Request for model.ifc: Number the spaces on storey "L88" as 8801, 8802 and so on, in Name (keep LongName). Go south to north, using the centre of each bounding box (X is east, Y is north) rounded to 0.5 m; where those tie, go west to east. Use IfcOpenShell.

First a look at what the model holds.

```python
import ifcopenshell
import ifcopenshell.util.element
import ifcopenshell.util.placement

model = ifcopenshell.open("model.ifc")
print(model.schema)
storey = next(s for s in model.by_type("IfcBuildingStorey") if s.Name == "L88")
spaces = [e for e in ifcopenshell.util.element.get_decomposition(storey) if e.is_a("IfcSpace")]
for e in sorted(spaces, key=lambda e: e.id()):
    origin = ifcopenshell.util.placement.get_local_placement(e.ObjectPlacement)[:3, 3]
    print(e.id(), e.Name, e.LongName, origin.round(2) + 0.0, sep=" | ")
```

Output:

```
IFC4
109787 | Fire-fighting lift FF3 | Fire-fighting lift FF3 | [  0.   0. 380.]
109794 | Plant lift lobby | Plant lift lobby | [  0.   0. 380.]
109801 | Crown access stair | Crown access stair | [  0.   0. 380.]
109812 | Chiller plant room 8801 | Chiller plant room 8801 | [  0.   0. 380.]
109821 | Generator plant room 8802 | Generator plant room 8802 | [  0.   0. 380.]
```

```python
import ifcopenshell
import ifcopenshell.geom
import ifcopenshell.util.element
import ifcopenshell.util.shape

model = ifcopenshell.open("model.ifc")
settings = ifcopenshell.geom.settings()
settings.set("use-world-coords", True)


def centre(element):
    shape = ifcopenshell.geom.create_shape(settings, element)
    return ifcopenshell.util.shape.get_bbox_centroid(shape.geometry)


storey = next(s for s in model.by_type("IfcBuildingStorey") if s.Name == "L88")
spaces = [e for e in ifcopenshell.util.element.get_decomposition(storey) if e.is_a("IfcSpace")]

# Insertion points can sit at a corner or the storey origin, so sort by the geometry (in metres).
centres = {e: centre(e) for e in spaces}
spaces.sort(key=lambda e: (round(centres[e][1] / 0.5), centres[e][0]))

for i, e in enumerate(spaces, start=1):
    number = f"88{i:02d}"
    e.Name = number
    print(e.id(), number)

model.write("model-out.ifc")
```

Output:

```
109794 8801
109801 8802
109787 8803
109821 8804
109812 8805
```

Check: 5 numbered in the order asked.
